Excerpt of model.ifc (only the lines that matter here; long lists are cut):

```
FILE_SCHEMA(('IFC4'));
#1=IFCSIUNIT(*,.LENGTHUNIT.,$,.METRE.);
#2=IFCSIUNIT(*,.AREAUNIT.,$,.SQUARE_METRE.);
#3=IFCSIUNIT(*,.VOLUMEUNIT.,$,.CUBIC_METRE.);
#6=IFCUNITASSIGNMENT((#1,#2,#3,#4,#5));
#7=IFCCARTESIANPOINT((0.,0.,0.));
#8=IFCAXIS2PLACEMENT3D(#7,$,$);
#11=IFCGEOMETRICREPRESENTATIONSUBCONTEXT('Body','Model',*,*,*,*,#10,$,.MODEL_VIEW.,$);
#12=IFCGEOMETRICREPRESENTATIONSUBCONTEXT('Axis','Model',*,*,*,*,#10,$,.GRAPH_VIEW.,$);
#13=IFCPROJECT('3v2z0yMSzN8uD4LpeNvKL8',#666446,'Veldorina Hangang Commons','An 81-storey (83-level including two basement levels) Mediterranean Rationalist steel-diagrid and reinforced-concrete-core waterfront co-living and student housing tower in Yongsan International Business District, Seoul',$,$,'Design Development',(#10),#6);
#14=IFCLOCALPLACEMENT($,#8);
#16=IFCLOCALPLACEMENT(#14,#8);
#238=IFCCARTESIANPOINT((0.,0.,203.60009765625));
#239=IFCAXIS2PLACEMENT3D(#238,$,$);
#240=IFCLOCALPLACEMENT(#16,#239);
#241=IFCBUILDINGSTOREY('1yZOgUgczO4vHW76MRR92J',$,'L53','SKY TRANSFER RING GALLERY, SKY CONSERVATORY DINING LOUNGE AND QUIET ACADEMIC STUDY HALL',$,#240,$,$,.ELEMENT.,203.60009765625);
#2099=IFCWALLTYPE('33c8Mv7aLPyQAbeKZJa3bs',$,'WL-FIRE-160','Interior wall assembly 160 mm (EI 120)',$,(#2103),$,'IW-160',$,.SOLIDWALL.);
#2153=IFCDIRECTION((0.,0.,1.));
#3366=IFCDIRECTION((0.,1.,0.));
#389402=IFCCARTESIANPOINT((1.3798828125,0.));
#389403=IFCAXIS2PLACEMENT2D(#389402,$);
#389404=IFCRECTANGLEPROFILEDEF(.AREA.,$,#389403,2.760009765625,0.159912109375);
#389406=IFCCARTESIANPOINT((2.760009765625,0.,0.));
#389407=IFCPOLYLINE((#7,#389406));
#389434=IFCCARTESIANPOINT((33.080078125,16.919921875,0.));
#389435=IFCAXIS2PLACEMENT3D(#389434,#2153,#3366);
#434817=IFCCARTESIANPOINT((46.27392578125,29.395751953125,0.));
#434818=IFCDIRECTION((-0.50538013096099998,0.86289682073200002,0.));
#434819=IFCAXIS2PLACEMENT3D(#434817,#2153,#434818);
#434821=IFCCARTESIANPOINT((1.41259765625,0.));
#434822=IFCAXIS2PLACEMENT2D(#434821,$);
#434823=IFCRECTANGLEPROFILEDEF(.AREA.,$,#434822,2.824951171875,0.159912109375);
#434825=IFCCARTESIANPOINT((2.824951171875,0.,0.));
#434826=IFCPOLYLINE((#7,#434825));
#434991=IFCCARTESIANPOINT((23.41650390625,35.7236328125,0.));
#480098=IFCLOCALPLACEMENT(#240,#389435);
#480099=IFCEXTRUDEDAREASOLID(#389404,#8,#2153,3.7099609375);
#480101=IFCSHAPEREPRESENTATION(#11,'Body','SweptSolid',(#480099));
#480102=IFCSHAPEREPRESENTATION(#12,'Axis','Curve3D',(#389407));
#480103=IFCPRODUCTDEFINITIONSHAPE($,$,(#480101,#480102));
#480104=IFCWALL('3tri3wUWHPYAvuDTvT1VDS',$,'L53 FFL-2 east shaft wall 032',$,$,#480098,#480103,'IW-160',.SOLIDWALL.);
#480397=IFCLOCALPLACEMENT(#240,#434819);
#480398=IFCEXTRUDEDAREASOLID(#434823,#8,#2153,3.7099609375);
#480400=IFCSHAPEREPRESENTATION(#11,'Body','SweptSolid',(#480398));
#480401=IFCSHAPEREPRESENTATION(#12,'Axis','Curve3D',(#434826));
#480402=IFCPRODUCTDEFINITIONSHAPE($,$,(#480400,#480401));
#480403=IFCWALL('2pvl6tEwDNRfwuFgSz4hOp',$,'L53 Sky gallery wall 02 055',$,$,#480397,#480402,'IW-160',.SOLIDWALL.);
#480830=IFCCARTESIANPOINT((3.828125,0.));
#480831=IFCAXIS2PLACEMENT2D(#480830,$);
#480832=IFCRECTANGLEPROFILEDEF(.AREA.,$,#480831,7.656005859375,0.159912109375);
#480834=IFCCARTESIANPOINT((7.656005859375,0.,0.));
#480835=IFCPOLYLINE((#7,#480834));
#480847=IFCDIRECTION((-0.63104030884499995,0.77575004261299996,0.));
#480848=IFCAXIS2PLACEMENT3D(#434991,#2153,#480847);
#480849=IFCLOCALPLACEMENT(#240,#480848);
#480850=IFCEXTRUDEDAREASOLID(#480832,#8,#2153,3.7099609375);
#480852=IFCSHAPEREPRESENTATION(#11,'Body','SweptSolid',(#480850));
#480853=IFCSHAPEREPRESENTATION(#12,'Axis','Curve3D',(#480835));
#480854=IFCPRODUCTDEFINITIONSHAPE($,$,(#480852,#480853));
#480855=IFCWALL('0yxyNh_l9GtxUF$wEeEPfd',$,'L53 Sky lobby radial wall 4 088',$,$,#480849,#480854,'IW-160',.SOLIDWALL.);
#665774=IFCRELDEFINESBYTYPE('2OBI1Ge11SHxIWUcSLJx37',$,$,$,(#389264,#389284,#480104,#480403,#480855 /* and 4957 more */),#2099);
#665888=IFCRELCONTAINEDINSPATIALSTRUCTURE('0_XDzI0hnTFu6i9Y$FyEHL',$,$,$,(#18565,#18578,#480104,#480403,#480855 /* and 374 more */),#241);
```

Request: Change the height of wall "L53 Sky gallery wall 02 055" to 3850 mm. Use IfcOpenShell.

```python
import ifcopenshell
import ifcopenshell.geom
import ifcopenshell.util.representation
import ifcopenshell.util.shape
import ifcopenshell.util.unit

model = ifcopenshell.open("model.ifc")
unit_scale = ifcopenshell.util.unit.calculate_unit_scale(model)
settings = ifcopenshell.geom.settings()


def volume(element):
    """Net volume in cubic metres, openings subtracted."""
    shape = ifcopenshell.geom.create_shape(settings, element)
    return ifcopenshell.util.shape.get_volume(shape.geometry)


wall = model.by_id(480403)
before = volume(wall)

body = ifcopenshell.util.representation.get_representation(wall, "Model", "Body")
solid = body.Items[0]
old_height = solid.Depth
solid.Depth = 3.85 / unit_scale
after = volume(wall)

print(f"height {old_height:g} -> {solid.Depth:g}, volume {before:.3f} -> {after:.3f} m3")

model.write("model_v2.ifc")
```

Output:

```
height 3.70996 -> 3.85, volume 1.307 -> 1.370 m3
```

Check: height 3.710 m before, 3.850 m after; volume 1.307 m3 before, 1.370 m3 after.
